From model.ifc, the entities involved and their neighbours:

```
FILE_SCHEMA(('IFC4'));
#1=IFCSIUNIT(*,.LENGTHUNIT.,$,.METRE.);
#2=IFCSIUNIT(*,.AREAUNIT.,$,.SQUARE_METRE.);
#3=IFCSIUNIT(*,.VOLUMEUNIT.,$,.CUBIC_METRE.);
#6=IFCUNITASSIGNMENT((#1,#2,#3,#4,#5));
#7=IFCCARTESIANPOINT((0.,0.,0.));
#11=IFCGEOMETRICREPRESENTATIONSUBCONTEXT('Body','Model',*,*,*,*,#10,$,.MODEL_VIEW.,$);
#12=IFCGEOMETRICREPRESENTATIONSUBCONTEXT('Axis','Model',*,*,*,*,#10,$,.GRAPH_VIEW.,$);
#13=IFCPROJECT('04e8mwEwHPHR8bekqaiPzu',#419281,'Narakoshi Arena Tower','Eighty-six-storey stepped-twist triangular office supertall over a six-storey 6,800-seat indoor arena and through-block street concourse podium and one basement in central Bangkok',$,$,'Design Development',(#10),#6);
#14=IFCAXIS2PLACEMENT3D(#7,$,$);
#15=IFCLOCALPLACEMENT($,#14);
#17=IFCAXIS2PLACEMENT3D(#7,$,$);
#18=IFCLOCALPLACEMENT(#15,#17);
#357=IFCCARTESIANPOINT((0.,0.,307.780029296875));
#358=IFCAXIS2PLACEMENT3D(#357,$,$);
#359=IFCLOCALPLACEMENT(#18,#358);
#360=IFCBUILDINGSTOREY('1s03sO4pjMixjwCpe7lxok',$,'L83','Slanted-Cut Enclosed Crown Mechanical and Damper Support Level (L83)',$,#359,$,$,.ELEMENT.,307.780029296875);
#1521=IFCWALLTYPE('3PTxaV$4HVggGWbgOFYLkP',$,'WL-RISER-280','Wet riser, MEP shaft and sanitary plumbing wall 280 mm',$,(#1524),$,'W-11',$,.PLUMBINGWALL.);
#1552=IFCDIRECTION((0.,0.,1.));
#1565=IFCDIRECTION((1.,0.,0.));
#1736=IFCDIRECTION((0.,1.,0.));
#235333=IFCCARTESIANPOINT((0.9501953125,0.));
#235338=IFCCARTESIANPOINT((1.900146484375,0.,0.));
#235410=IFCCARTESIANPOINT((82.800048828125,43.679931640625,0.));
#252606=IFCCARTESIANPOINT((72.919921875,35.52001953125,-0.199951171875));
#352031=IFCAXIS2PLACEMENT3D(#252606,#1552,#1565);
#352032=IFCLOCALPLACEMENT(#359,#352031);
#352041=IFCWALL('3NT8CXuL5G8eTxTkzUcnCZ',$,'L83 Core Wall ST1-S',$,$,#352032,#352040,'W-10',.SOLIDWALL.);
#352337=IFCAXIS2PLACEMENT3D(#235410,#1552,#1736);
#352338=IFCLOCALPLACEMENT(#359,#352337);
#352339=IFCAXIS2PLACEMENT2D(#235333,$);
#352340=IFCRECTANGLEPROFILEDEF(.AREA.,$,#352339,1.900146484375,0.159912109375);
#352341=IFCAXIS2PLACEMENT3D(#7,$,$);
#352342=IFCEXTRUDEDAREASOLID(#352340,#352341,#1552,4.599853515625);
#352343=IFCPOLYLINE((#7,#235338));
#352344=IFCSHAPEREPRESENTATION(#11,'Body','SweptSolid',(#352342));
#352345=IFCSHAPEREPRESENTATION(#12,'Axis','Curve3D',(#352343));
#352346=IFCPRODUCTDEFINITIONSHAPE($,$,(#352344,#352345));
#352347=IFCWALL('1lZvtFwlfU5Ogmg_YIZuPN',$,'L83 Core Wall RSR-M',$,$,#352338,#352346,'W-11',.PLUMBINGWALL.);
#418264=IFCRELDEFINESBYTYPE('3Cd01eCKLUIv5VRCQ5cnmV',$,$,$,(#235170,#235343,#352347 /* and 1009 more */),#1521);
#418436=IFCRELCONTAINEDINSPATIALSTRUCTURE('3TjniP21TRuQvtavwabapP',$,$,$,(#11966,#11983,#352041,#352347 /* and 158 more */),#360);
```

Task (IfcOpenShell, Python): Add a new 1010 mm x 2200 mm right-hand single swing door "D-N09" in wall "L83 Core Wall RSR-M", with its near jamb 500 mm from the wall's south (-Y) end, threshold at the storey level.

```python
import numpy as np
import ifcopenshell
import ifcopenshell.api.feature
import ifcopenshell.api.geometry
import ifcopenshell.api.root
import ifcopenshell.api.spatial
import ifcopenshell.geom
import ifcopenshell.util.element
import ifcopenshell.util.placement
import ifcopenshell.util.representation
import ifcopenshell.util.shape
import ifcopenshell.util.unit

model = ifcopenshell.open("model.ifc")
unit_scale = ifcopenshell.util.unit.calculate_unit_scale(model)
settings = ifcopenshell.geom.settings()


def volume(element):
    """Net volume in cubic metres, openings subtracted."""
    shape = ifcopenshell.geom.create_shape(settings, element)
    return ifcopenshell.util.shape.get_volume(shape.geometry)


wall = model.by_guid("1lZvtFwlfU5Ogmg_YIZuPN")
storey = ifcopenshell.util.element.get_container(wall, ifc_class="IfcBuildingStorey")
context = ifcopenshell.util.representation.get_context(model, "Model", "Body", "MODEL_VIEW")
before = volume(wall)

width, height, from_end, sill = 1.01, 2.2, 0.5, 0.0  # metres

# The wall runs along its own X axis, and the end named is its -X end.
wall_shape = ifcopenshell.geom.create_shape(settings, wall)
x, y, z = ifcopenshell.util.shape.get_vertices(wall_shape.geometry).T
start = x.min() + from_end
face, thickness = float(y.min()), float(y.max() - y.min())
wall_matrix = ifcopenshell.util.placement.get_local_placement(wall.ObjectPlacement)
level = ifcopenshell.util.placement.get_local_placement(storey.ObjectPlacement)[2, 3]


def in_wall(x, y):
    """Placement at x, y metres in the wall's axes, at sill height."""
    matrix = wall_matrix.copy()
    matrix[:, 3] = wall_matrix @ np.array([x / unit_scale, y / unit_scale, 0.0, 1.0])
    matrix[2, 3] = level + sill / unit_scale
    return matrix


# Opening: a box that overshoots both wall faces by 50 mm.
opening = ifcopenshell.api.root.create_entity(model, ifc_class="IfcOpeningElement", predefined_type="OPENING")
box = ifcopenshell.api.geometry.add_wall_representation(
    model, context=context, length=width, height=height, thickness=thickness + 0.1
)
ifcopenshell.api.geometry.assign_representation(model, product=opening, representation=box)
ifcopenshell.api.geometry.edit_object_placement(model, product=opening, matrix=in_wall(start, face - 0.05), is_si=False)
ifcopenshell.api.feature.add_feature(model, feature=opening, element=wall)

door = ifcopenshell.api.root.create_entity(model, ifc_class="IfcDoor", name="D-N09", predefined_type="DOOR")
door.OverallWidth, door.OverallHeight = width / unit_scale, height / unit_scale
door.OperationType = "SINGLE_SWING_RIGHT"
body = ifcopenshell.api.geometry.add_door_representation(
    model,
    context=context,
    overall_width=door.OverallWidth,
    overall_height=door.OverallHeight,
    operation_type="SINGLE_SWING_RIGHT",
    lining_properties={"LiningDepth": thickness / unit_scale, "ThresholdDepth": thickness / unit_scale},
)
ifcopenshell.api.geometry.assign_representation(model, product=door, representation=body)
ifcopenshell.api.spatial.assign_container(model, products=[door], relating_structure=storey)
ifcopenshell.api.feature.add_filling(model, opening=opening, element=door)

# The lining spans the wall, so the door starts at the wall face.
ifcopenshell.api.geometry.edit_object_placement(model, product=door, matrix=in_wall(start, face), is_si=False)

after = volume(wall)

print(f"wall volume {before:.3f} -> {after:.3f} m3")

model.write("model_updated.ifc")
```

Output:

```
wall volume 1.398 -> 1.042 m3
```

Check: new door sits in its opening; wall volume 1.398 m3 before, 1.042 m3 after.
